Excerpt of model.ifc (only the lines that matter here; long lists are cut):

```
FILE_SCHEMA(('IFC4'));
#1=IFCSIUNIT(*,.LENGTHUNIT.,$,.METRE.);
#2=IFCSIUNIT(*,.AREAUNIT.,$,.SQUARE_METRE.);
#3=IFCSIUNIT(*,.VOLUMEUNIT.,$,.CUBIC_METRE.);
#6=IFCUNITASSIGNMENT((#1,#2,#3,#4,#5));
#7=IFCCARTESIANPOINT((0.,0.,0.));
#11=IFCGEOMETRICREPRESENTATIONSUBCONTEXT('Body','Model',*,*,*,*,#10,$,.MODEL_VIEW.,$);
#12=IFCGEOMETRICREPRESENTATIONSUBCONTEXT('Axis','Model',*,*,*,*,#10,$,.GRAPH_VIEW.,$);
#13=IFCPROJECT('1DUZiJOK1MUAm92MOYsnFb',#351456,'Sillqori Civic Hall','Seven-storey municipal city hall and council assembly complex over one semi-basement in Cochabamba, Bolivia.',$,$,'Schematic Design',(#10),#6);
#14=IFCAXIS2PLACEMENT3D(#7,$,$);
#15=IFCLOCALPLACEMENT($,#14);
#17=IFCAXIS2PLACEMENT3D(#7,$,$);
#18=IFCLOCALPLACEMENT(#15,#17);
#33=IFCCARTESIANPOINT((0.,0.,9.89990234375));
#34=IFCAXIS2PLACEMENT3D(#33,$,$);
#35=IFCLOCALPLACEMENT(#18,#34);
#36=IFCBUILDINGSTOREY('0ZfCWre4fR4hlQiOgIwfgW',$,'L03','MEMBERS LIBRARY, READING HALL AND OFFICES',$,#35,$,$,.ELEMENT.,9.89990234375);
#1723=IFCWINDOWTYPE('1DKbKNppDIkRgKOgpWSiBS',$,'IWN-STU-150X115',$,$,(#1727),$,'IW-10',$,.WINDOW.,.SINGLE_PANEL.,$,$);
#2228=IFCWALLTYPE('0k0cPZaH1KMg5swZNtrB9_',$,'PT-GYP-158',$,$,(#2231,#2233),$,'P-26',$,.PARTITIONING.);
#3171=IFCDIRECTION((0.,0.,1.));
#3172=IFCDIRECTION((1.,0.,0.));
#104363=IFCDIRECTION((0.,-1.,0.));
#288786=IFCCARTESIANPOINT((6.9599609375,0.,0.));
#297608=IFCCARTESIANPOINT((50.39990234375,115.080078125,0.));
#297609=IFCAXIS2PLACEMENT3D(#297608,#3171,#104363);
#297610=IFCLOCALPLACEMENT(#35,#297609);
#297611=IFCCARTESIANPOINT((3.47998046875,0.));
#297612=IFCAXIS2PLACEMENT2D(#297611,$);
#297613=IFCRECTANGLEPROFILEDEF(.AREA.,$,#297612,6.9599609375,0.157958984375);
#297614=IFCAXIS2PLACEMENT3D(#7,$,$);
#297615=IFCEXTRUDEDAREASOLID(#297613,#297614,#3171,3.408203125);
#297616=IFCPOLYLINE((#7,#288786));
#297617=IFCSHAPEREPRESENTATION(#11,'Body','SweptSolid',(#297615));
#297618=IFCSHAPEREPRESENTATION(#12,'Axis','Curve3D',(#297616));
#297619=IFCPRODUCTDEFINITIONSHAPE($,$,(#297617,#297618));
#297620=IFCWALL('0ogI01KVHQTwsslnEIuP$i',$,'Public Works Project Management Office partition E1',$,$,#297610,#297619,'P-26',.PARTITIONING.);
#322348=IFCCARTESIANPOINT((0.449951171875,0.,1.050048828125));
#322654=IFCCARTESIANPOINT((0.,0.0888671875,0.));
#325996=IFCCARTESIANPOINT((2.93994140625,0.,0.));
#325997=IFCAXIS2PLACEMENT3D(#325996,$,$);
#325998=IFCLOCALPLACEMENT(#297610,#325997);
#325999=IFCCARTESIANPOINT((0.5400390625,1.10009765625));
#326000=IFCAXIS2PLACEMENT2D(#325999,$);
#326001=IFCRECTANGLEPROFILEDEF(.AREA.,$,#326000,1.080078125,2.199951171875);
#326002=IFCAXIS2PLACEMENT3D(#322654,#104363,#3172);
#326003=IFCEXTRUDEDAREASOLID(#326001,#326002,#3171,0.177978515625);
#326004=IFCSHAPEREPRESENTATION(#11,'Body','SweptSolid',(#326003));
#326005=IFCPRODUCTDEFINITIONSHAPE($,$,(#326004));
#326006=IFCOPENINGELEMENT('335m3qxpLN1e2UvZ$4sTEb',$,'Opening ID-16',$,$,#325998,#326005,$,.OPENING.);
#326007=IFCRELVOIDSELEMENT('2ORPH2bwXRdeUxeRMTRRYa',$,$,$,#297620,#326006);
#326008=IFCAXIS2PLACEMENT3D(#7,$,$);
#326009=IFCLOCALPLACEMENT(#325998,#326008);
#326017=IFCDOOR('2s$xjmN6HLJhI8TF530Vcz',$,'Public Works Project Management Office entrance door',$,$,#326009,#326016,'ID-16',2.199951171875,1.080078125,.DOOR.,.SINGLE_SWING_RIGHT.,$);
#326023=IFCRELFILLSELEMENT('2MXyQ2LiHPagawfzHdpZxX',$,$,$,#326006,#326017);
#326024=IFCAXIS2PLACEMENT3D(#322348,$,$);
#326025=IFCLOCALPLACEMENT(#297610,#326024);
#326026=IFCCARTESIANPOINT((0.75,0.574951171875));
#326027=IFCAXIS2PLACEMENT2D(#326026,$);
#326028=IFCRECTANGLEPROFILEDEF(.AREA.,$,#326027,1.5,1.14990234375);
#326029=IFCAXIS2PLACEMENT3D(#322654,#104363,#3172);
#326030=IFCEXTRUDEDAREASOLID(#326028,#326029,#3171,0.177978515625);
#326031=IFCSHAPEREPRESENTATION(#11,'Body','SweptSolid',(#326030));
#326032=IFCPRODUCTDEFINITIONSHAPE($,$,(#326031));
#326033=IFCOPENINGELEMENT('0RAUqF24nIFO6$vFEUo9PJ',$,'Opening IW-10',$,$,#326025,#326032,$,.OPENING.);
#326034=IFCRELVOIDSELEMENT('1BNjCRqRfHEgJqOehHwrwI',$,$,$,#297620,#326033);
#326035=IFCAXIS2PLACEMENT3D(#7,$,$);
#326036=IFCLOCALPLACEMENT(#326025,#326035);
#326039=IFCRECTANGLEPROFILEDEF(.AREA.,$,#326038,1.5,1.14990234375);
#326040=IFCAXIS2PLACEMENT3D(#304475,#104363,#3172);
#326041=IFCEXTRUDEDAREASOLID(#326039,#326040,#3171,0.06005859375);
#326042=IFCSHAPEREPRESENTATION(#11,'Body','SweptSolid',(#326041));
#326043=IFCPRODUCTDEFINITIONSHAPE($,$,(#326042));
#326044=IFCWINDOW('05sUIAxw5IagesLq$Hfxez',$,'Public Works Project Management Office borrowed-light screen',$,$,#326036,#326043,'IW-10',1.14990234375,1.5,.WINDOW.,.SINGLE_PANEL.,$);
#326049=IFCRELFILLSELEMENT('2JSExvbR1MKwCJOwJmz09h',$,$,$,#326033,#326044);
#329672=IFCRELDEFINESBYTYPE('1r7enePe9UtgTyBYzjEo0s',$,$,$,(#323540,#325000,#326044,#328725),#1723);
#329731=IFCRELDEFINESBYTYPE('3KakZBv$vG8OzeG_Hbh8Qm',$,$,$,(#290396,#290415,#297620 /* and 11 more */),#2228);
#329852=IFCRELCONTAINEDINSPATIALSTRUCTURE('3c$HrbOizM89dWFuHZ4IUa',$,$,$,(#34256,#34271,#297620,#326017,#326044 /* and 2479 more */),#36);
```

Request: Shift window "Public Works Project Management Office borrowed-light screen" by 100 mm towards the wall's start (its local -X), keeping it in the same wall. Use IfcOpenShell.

```python
import ifcopenshell
import ifcopenshell.api.geometry
import ifcopenshell.util.placement
import ifcopenshell.util.unit

model = ifcopenshell.open("model.ifc")
unit_scale = ifcopenshell.util.unit.calculate_unit_scale(model)

window = model.by_guid("05sUIAxw5IagesLq$Hfxez")
opening = window.FillsVoids[0].RelatingOpeningElement
wall = opening.VoidsElements[0].RelatingBuildingElement

wall_matrix = ifcopenshell.util.placement.get_local_placement(wall.ObjectPlacement)
shift = wall_matrix[:3, 0] * -0.1 / unit_scale
before = ifcopenshell.util.placement.get_local_placement(window.ObjectPlacement)[:3, 3].copy()

# The window is placed relative to its opening, so it follows when the opening moves.
matrix = ifcopenshell.util.placement.get_local_placement(opening.ObjectPlacement)
matrix[:3, 3] += shift
ifcopenshell.api.geometry.edit_object_placement(
    model, product=opening, matrix=matrix, is_si=False, should_transform_children=True
)

after = ifcopenshell.util.placement.get_local_placement(window.ObjectPlacement)[:3, 3]
print("window moved by", (after - before).round(3) + 0.0)

model.write("model_updated.ifc")
```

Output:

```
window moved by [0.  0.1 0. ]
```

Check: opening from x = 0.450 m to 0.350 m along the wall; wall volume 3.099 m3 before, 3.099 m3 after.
